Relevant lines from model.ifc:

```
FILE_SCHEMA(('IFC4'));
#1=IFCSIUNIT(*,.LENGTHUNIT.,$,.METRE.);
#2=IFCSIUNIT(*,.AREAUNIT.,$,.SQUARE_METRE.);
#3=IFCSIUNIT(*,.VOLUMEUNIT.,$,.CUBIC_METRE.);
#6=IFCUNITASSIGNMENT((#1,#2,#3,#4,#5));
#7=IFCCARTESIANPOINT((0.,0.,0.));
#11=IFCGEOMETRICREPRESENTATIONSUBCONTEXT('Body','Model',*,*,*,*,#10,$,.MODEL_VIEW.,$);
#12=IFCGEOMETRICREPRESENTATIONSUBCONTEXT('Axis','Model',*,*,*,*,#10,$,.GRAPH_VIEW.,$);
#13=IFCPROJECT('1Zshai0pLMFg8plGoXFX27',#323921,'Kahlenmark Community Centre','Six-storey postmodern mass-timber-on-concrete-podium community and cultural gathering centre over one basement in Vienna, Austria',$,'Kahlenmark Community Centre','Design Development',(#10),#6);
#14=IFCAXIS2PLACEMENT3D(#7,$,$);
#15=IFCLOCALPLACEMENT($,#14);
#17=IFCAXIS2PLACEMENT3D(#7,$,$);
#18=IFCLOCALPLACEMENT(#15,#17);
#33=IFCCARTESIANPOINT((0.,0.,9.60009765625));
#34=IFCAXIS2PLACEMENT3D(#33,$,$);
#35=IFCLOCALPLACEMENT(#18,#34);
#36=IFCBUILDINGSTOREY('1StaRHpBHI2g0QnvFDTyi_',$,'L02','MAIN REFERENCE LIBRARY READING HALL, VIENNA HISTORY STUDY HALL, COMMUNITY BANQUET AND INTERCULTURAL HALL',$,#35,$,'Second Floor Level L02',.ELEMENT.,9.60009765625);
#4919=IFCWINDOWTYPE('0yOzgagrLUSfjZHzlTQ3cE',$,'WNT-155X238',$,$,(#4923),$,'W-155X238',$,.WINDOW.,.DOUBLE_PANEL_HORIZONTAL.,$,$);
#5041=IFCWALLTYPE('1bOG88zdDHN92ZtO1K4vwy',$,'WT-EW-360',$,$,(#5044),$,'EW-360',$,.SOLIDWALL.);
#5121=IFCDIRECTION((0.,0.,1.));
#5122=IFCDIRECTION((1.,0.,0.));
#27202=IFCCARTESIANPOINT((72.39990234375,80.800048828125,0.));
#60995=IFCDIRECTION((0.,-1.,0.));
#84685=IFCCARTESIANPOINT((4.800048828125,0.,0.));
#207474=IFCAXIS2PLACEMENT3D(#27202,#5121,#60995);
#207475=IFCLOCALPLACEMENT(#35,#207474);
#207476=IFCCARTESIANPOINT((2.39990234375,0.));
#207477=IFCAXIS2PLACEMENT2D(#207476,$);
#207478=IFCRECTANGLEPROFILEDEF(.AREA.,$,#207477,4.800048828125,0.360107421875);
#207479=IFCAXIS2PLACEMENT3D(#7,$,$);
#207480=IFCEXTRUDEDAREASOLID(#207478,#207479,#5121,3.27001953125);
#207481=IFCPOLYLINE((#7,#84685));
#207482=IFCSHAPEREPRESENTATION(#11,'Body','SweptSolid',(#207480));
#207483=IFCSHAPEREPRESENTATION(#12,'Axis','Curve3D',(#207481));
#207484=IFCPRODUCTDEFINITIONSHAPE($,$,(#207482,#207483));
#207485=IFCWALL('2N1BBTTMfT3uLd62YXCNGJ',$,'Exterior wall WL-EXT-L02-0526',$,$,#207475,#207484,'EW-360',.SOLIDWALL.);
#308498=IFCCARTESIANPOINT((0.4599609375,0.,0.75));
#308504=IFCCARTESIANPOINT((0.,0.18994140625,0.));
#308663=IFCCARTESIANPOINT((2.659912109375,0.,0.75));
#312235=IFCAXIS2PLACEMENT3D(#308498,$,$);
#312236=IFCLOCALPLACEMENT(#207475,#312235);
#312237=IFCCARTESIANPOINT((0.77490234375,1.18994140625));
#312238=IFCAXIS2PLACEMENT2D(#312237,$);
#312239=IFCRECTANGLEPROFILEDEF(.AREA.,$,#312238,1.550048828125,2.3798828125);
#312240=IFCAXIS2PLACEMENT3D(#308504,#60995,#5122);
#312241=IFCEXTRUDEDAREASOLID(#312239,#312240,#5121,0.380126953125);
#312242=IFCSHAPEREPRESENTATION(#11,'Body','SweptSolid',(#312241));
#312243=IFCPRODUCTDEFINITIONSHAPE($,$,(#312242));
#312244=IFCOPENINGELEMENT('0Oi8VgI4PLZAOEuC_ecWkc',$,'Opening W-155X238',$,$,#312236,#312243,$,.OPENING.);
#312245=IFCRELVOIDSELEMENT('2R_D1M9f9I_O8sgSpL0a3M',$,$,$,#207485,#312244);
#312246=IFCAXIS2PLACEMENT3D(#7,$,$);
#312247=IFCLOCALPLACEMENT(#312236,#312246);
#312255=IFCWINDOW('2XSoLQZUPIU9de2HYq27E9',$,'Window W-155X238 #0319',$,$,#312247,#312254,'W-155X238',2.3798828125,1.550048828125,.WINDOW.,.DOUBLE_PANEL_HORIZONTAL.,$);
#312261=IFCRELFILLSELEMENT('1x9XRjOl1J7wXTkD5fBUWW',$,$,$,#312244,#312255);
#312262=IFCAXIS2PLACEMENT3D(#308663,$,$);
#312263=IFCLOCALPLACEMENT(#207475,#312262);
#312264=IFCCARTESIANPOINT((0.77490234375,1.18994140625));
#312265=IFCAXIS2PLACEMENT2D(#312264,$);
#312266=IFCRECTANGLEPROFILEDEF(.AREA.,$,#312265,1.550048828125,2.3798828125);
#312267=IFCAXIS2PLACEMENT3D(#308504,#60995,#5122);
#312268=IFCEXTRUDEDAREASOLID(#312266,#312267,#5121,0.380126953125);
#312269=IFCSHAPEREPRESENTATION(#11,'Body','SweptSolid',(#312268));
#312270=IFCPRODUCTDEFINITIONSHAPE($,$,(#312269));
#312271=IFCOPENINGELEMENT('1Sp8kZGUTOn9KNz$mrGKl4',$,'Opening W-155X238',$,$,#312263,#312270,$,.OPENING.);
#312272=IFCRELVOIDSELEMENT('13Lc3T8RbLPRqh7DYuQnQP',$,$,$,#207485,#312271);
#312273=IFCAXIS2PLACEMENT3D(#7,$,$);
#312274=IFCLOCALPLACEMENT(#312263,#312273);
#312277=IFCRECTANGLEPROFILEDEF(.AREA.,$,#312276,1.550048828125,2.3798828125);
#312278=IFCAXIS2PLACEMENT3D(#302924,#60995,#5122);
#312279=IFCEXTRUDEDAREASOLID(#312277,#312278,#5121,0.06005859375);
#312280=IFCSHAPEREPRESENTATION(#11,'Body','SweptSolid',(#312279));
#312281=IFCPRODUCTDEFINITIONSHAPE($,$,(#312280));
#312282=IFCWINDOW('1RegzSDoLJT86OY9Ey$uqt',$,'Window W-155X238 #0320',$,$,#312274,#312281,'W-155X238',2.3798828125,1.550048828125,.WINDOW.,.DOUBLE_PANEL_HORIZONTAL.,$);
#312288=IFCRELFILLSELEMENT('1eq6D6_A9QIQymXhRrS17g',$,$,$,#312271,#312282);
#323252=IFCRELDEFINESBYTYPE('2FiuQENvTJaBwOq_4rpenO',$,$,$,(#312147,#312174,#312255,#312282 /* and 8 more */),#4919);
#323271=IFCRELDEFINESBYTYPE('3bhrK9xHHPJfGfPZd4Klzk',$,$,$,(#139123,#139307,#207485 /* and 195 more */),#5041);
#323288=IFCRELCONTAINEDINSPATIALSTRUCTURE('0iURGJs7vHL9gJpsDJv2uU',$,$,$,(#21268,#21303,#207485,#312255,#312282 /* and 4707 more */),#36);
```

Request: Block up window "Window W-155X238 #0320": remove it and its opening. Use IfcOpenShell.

```python
import ifcopenshell
import ifcopenshell.api.feature
import ifcopenshell.api.root
import ifcopenshell.geom
import ifcopenshell.util.shape

model = ifcopenshell.open("model.ifc")
settings = ifcopenshell.geom.settings()


def volume(element):
    """Net volume in cubic metres, openings subtracted."""
    shape = ifcopenshell.geom.create_shape(settings, element)
    return ifcopenshell.util.shape.get_volume(shape.geometry)


window = model.by_id(312282)
opening = window.FillsVoids[0].RelatingOpeningElement
wall = opening.VoidsElements[0].RelatingBuildingElement
before = volume(wall)

ifcopenshell.api.root.remove_product(model, product=window)
ifcopenshell.api.feature.remove_feature(model, feature=opening)

after = volume(wall)

print(f"wall volume {before:.3f} -> {after:.3f} m3")

model.write("model_v2.ifc")
```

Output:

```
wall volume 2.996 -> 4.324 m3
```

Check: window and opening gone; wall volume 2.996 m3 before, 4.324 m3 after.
